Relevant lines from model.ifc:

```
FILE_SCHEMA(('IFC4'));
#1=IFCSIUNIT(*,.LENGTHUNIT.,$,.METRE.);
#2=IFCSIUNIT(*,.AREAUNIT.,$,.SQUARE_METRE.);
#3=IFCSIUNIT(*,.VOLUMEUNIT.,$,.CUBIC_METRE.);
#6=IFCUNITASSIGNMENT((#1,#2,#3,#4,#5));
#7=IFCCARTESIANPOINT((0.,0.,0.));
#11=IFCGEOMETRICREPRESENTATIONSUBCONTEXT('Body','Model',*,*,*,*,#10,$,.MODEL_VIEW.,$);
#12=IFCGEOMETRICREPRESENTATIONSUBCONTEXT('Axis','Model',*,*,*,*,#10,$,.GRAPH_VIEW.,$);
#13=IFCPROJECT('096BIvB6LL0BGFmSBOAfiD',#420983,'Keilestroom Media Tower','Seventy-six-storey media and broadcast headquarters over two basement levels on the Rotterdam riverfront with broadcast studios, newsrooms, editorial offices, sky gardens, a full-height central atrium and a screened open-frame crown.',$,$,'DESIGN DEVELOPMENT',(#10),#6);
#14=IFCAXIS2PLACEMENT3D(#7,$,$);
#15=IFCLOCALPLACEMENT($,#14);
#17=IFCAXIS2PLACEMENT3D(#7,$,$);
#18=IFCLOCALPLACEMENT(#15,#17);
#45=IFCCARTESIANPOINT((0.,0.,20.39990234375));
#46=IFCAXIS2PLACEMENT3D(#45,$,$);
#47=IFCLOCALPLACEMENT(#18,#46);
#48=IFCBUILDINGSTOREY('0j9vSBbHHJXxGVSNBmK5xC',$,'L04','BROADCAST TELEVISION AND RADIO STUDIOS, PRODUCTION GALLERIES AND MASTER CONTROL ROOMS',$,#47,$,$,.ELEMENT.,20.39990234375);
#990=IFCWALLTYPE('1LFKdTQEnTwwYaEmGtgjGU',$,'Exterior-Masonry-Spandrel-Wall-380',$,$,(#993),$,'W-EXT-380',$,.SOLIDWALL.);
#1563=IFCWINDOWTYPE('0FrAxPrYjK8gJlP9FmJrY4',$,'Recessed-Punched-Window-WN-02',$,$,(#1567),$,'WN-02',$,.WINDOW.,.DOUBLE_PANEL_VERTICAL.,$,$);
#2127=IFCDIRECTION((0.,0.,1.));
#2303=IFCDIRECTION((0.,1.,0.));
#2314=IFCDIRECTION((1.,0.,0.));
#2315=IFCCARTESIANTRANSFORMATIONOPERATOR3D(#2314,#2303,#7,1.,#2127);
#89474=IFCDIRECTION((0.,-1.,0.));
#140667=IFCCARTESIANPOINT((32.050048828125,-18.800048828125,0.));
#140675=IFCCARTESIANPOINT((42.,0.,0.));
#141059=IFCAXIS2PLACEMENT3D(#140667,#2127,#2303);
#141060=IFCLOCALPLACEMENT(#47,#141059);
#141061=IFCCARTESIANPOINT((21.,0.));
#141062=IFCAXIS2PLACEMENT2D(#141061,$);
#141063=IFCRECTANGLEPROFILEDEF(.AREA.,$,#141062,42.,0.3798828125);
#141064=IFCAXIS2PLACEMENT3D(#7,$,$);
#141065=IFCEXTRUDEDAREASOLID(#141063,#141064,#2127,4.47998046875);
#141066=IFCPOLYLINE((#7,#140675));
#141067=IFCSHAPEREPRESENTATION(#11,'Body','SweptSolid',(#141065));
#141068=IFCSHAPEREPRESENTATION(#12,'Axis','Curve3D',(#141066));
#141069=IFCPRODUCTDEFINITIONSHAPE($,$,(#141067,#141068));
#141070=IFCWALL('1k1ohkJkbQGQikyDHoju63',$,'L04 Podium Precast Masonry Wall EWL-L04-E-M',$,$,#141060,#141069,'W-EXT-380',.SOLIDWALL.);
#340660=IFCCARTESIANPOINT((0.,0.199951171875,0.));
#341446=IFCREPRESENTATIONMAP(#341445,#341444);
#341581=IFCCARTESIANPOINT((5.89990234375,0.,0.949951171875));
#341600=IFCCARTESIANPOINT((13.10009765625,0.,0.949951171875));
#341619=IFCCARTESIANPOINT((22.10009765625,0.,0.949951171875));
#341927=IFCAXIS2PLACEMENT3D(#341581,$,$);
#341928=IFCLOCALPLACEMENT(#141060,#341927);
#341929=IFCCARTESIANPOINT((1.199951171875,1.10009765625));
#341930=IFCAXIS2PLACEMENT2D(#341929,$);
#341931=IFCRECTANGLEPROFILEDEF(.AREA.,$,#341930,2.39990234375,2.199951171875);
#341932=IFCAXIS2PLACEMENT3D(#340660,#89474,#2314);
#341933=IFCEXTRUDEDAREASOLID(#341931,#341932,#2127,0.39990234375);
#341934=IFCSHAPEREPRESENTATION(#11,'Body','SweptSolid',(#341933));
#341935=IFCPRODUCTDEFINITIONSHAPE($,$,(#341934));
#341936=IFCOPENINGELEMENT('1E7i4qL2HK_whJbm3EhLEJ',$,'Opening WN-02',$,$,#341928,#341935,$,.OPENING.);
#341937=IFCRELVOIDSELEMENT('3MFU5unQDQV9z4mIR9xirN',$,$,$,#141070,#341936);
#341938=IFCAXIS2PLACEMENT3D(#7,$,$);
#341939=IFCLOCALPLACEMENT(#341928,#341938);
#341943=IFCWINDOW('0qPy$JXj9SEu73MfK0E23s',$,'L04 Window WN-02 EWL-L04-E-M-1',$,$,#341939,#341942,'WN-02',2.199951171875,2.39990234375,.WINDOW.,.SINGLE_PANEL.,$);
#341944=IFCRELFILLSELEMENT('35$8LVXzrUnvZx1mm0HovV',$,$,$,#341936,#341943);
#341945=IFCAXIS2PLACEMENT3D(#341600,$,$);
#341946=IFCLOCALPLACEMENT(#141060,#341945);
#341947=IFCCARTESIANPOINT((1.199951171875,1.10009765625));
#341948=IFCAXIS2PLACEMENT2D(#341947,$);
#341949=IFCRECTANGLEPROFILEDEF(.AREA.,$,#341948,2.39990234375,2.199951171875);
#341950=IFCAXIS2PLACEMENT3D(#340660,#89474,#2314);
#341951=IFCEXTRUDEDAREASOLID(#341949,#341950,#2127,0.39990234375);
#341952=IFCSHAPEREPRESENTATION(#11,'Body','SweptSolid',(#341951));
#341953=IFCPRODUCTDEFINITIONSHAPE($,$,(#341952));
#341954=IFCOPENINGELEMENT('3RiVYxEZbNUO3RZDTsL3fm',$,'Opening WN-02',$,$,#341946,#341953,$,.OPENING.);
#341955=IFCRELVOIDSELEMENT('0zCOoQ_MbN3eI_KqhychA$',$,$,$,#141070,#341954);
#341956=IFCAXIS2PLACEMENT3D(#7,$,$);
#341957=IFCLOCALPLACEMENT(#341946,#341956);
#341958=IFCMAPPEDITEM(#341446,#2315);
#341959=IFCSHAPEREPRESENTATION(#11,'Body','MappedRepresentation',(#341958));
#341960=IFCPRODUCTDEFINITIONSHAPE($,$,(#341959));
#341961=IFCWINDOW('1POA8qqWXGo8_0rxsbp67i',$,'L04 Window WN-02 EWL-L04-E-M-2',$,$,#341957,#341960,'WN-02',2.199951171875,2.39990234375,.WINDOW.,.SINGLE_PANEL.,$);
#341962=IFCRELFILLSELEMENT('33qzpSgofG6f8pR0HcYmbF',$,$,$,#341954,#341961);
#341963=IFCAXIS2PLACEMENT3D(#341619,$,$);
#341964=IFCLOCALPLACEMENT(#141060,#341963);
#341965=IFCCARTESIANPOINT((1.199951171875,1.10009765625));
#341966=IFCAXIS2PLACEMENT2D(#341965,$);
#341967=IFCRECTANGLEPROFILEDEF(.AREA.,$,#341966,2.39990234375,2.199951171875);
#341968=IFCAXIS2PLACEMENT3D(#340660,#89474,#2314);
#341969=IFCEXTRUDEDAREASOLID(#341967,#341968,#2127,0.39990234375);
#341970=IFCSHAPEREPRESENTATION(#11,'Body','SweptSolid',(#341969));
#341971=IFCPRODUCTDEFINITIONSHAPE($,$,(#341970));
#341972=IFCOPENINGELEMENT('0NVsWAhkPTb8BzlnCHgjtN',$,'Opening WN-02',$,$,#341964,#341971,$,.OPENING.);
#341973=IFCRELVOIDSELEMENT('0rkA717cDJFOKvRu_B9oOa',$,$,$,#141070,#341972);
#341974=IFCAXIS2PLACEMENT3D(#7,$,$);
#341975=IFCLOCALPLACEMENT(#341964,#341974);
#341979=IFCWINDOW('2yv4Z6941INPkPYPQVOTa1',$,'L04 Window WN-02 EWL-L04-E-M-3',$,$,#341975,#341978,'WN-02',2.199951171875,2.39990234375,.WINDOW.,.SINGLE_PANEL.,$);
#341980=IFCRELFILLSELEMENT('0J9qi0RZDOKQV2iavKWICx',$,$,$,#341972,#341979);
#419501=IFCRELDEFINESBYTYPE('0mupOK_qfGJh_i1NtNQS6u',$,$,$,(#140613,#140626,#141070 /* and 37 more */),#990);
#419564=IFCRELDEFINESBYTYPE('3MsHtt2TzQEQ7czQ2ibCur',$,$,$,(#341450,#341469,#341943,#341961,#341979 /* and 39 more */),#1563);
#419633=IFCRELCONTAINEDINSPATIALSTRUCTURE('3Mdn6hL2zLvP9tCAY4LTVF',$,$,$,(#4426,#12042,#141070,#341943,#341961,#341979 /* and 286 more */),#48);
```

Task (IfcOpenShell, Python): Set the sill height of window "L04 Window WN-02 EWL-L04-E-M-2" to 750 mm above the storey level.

```python
import numpy as np
import ifcopenshell
import ifcopenshell.api.geometry
import ifcopenshell.geom
import ifcopenshell.util.element
import ifcopenshell.util.placement
import ifcopenshell.util.shape
import ifcopenshell.util.unit

model = ifcopenshell.open("model.ifc")
unit_scale = ifcopenshell.util.unit.calculate_unit_scale(model)

window = model.by_guid("1POA8qqWXGo8_0rxsbp67i")
opening = window.FillsVoids[0].RelatingOpeningElement
storey = ifcopenshell.util.element.get_container(window, ifc_class="IfcBuildingStorey")
level = ifcopenshell.util.placement.get_local_placement(storey.ObjectPlacement)[2, 3]

# The opening's origin need not be at the sill, so measure its lowest point.
shape = ifcopenshell.geom.create_shape(ifcopenshell.geom.settings(), opening)
bottom = ifcopenshell.util.shape.get_shape_bottom_elevation(shape, shape.geometry) / unit_scale
dz = level + 0.75 - bottom

shift = np.array([0.0, 0.0, dz])
# The window is placed relative to its opening, so it follows when the opening moves.
matrix = ifcopenshell.util.placement.get_local_placement(opening.ObjectPlacement)
matrix[:3, 3] += shift
ifcopenshell.api.geometry.edit_object_placement(
    model, product=opening, matrix=matrix, is_si=False, should_transform_children=True
)

print(f"moved by {dz * unit_scale:+.3f} m")

model.write("model_v2.ifc")
```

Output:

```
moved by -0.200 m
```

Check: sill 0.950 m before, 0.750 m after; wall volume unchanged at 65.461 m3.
